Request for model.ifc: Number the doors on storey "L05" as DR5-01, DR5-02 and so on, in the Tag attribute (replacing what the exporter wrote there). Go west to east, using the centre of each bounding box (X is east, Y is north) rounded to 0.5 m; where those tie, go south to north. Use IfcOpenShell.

First a look at what the model holds.

```python
import ifcopenshell
import ifcopenshell.util.element
import ifcopenshell.util.placement

model = ifcopenshell.open("model.ifc")
print(model.schema)
storey = next(s for s in model.by_type("IfcBuildingStorey") if s.Name == "L05")
doors = [e for e in ifcopenshell.util.element.get_decomposition(storey) if e.is_a("IfcDoor")]
for e in sorted(doors, key=lambda e: e.id()):
    origin = ifcopenshell.util.placement.get_local_placement(e.ObjectPlacement)[:3, 3]
    print(e.id(), e.Tag, e.Name, origin.round(2) + 0.0, sep=" | ")
```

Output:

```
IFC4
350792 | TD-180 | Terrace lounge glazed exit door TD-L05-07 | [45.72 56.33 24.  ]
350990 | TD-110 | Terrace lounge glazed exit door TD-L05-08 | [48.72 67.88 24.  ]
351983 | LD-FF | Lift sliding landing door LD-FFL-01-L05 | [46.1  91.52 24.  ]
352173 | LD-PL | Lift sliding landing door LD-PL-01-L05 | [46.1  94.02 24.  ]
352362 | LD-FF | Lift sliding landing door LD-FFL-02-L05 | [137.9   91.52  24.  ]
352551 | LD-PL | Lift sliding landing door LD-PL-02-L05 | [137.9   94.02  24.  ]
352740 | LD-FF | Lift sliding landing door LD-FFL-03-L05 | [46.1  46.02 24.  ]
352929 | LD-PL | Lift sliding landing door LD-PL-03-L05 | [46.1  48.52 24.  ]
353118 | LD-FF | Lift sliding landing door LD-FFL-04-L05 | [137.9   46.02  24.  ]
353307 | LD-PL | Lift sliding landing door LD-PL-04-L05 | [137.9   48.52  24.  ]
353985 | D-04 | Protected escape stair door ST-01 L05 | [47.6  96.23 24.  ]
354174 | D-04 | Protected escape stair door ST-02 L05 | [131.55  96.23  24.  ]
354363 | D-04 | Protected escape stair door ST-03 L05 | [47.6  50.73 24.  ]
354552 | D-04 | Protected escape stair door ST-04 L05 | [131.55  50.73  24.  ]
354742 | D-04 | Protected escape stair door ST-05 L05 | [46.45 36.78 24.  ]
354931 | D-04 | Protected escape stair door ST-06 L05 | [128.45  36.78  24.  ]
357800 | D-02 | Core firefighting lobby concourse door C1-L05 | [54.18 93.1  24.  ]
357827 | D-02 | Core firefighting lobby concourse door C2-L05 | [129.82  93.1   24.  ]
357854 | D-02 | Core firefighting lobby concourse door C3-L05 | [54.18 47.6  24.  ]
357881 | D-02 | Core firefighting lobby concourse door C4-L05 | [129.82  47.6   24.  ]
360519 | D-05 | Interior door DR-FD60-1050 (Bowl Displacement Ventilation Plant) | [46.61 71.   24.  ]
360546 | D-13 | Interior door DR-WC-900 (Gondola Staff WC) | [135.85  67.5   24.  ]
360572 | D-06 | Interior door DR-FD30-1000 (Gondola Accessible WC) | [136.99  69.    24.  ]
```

```python
import ifcopenshell
import ifcopenshell.geom
import ifcopenshell.util.element
import ifcopenshell.util.shape

model = ifcopenshell.open("model.ifc")
settings = ifcopenshell.geom.settings()
settings.set("use-world-coords", True)


def centre(element):
    shape = ifcopenshell.geom.create_shape(settings, element)
    return ifcopenshell.util.shape.get_bbox_centroid(shape.geometry)


storey = next(s for s in model.by_type("IfcBuildingStorey") if s.Name == "L05")
doors = [e for e in ifcopenshell.util.element.get_decomposition(storey) if e.is_a("IfcDoor")]

# Insertion points can sit at a corner or the storey origin, so sort by the geometry (in metres).
centres = {e: centre(e) for e in doors}
doors.sort(key=lambda e: (round(centres[e][0] / 0.5), centres[e][1]))

for i, e in enumerate(doors, start=1):
    number = f"DR5-{i:02d}"
    e.Tag = number
    print(e.id(), number)

model.write("model-out.ifc")
```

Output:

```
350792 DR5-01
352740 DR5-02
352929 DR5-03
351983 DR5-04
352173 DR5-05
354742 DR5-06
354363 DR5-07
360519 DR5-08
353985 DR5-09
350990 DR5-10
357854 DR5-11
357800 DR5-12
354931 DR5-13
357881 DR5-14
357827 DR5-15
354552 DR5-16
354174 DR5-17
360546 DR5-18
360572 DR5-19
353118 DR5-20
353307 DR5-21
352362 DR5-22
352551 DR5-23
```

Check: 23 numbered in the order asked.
